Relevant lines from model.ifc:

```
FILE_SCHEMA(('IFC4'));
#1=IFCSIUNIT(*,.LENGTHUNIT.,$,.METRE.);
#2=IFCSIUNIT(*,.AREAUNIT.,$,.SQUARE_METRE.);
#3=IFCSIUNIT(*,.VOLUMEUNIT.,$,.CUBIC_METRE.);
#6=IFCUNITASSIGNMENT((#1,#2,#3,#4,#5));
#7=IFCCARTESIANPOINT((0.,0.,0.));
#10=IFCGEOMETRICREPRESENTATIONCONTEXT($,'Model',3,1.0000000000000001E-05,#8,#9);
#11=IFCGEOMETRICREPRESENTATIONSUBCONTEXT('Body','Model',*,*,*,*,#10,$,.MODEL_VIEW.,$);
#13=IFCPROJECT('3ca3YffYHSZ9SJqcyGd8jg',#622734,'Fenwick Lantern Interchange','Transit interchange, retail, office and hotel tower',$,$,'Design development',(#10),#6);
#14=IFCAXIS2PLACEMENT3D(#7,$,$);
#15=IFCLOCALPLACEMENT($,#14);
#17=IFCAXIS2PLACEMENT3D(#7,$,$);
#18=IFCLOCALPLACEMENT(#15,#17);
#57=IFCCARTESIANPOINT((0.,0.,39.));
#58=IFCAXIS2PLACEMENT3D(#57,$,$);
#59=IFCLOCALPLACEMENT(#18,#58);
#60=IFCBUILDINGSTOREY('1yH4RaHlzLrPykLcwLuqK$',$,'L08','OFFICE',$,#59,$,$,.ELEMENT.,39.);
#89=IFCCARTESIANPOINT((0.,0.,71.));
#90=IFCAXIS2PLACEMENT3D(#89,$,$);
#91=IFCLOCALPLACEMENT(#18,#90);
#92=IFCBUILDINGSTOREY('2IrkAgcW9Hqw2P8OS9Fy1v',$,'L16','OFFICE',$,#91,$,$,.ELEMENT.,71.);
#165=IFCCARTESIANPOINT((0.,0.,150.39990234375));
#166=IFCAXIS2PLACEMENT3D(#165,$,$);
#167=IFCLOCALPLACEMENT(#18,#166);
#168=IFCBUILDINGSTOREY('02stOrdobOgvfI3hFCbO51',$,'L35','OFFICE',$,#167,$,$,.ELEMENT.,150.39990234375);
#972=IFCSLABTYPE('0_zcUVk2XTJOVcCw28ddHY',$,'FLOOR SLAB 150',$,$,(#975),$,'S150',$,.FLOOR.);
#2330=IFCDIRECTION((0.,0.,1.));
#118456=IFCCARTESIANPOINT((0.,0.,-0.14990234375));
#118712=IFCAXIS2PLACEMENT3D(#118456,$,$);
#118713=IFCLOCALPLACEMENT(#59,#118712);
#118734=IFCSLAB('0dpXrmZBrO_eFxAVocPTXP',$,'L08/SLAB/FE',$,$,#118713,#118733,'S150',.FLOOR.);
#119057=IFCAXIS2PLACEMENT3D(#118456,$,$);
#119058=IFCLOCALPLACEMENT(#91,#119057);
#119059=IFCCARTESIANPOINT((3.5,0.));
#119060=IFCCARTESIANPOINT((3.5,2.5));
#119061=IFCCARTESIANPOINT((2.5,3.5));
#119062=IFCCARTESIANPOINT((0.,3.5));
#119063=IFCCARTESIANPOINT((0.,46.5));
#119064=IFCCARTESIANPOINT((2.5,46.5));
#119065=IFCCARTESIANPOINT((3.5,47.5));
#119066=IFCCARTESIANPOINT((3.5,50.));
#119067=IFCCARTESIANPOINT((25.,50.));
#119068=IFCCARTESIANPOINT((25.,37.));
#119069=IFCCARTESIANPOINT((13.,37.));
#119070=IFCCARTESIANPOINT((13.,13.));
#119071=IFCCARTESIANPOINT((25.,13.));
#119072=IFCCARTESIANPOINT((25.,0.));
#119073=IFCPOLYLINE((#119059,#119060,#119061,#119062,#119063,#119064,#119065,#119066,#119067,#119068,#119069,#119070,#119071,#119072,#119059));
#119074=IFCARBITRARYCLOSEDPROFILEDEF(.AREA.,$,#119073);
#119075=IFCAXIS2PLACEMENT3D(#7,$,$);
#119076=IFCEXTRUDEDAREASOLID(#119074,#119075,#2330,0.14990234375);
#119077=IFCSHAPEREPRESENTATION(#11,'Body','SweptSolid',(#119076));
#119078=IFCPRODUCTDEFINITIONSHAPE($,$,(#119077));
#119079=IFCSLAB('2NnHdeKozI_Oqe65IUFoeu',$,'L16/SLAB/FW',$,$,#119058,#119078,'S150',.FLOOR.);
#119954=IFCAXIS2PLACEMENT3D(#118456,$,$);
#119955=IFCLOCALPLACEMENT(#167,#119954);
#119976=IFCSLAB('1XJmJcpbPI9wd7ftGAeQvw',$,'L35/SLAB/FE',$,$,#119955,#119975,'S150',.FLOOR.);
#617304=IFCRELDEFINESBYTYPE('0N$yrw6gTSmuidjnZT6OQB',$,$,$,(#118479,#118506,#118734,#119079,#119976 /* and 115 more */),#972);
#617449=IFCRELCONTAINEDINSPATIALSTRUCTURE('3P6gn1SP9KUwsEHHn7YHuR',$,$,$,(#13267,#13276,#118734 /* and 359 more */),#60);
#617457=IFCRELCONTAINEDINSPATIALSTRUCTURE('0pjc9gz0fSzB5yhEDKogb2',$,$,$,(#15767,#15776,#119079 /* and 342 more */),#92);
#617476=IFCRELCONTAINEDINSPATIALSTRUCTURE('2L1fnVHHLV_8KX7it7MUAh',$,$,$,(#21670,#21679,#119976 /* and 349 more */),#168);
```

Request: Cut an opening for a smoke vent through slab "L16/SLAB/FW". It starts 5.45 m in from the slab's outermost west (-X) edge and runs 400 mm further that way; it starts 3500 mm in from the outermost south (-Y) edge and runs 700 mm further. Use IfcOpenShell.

```python
import numpy as np
import ifcopenshell
import ifcopenshell.api.feature
import ifcopenshell.api.geometry
import ifcopenshell.api.root
import ifcopenshell.geom
import ifcopenshell.util.placement
import ifcopenshell.util.representation
import ifcopenshell.util.shape
import ifcopenshell.util.unit

model = ifcopenshell.open("model.ifc")
unit_scale = ifcopenshell.util.unit.calculate_unit_scale(model)
settings = ifcopenshell.geom.settings()


def volume(element):
    """Net volume in cubic metres, openings subtracted."""
    shape = ifcopenshell.geom.create_shape(settings, element)
    return ifcopenshell.util.shape.get_volume(shape.geometry)


slab = model.by_guid("2NnHdeKozI_Oqe65IUFoeu")
before = volume(slab)

# Extent in the slab's own axes, in metres. The edges named are its -X and -Y sides.
slab_shape = ifcopenshell.geom.create_shape(settings, slab)
vertices = ifcopenshell.util.shape.get_vertices(slab_shape.geometry)
x_min, y_min, bottom = vertices.min(axis=0)
top = vertices[:, 2].max()

opening = ifcopenshell.api.root.create_entity(model, ifc_class="IfcOpeningElement", name="Smoke vent opening", predefined_type="OPENING")
context = ifcopenshell.util.representation.get_context(model, "Model", "Body", "MODEL_VIEW")
width, depth = 0.4, 0.7
outline = [(0.0, 0.0), (width, 0.0), (width, depth), (0.0, depth), (0.0, 0.0)]
# Overshoot both faces by 50 mm so the cut is clean.
shape = ifcopenshell.api.geometry.add_slab_representation(
    model, context=context, depth=top - bottom + 0.1, polyline=outline
)
ifcopenshell.api.geometry.assign_representation(model, product=opening, representation=shape)

matrix = ifcopenshell.util.placement.get_local_placement(slab.ObjectPlacement)
matrix[:, 3] = matrix @ np.append(np.array([x_min + 5.45, y_min + 3.5, bottom - 0.05]) / unit_scale, 1.0)
ifcopenshell.api.geometry.edit_object_placement(model, product=opening, matrix=matrix, is_si=False)
ifcopenshell.api.feature.add_feature(model, feature=opening, element=slab)

after = volume(slab)

print(f"slab volume {before:.3f} -> {after:.3f} m3")

model.write("model_updated.ifc")
```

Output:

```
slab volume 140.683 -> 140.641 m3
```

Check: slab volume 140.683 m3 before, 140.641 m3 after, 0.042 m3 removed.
